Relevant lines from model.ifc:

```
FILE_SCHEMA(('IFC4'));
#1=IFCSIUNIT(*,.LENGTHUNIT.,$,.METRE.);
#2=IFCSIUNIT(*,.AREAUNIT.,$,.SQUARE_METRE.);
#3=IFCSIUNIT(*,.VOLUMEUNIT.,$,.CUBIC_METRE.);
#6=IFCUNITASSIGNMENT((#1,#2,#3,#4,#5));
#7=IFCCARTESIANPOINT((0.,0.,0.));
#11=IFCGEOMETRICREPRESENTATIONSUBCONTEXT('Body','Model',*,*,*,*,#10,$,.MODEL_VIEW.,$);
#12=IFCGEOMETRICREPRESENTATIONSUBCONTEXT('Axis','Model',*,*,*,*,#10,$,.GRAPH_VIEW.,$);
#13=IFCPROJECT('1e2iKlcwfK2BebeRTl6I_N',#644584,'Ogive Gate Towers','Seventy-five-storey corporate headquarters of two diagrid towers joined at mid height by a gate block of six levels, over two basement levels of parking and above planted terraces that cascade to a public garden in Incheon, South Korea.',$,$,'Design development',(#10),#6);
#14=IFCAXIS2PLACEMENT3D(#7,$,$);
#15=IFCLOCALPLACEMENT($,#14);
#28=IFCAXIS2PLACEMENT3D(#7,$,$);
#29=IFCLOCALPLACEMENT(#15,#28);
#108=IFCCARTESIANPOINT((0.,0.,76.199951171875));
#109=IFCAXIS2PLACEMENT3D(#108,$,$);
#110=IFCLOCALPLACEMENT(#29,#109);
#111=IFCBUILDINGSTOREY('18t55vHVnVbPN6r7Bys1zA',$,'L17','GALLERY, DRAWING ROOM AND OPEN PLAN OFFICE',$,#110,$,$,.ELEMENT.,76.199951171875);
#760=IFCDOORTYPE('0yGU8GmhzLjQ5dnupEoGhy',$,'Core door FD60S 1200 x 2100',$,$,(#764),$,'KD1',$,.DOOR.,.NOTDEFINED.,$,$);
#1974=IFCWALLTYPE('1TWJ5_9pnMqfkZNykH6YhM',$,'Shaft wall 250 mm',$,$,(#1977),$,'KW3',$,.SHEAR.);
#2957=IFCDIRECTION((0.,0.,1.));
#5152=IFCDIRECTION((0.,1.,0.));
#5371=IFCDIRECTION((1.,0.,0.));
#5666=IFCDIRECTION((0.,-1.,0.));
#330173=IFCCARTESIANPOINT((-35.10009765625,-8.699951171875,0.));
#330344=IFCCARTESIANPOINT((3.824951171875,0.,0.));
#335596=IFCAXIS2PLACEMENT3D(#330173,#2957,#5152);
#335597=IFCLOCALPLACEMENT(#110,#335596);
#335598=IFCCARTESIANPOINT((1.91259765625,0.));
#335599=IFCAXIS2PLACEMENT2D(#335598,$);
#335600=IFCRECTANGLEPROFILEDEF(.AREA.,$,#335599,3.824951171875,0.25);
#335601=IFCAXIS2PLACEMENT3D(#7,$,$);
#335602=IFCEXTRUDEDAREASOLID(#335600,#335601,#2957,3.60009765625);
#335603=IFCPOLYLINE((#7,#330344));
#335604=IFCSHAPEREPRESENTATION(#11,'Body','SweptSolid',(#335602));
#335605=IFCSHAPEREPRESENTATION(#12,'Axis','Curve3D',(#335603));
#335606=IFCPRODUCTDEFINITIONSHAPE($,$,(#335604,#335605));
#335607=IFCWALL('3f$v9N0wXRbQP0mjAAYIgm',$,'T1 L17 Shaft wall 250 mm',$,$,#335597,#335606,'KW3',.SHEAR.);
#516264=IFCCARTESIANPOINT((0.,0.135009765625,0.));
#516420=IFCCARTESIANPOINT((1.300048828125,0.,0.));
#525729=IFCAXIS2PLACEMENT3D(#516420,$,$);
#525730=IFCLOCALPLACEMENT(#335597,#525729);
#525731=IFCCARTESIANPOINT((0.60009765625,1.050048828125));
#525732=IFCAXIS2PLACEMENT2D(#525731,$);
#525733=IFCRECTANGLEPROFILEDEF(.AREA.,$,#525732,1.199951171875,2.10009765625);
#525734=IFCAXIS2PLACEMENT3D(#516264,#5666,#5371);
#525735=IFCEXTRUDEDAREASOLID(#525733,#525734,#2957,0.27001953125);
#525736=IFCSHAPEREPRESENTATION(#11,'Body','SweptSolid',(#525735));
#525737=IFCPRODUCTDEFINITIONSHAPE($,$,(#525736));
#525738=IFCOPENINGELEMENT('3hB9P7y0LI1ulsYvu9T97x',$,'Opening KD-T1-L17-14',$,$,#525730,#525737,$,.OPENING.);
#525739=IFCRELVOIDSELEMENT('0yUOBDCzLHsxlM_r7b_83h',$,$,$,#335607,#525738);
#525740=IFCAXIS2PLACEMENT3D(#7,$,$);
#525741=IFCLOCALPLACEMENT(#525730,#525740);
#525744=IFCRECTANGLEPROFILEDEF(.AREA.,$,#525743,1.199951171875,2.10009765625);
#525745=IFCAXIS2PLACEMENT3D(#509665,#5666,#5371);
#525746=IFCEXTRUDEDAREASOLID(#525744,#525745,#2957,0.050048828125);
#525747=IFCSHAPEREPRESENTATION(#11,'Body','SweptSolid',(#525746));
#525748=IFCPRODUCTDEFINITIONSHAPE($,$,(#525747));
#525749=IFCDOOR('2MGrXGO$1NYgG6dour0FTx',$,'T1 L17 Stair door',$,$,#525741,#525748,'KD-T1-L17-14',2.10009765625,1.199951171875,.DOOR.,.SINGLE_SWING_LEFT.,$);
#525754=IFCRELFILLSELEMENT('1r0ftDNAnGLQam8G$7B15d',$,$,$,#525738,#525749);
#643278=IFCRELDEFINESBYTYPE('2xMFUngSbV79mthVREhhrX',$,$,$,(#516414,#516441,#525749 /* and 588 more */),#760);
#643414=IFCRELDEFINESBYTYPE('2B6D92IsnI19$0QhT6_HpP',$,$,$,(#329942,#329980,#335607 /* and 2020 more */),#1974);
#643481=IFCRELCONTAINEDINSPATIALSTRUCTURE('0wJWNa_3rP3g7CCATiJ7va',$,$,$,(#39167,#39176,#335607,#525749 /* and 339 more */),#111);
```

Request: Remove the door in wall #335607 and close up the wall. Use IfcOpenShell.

```python
import ifcopenshell
import ifcopenshell.api.feature
import ifcopenshell.api.root
import ifcopenshell.geom
import ifcopenshell.util.shape

model = ifcopenshell.open("model.ifc")
settings = ifcopenshell.geom.settings()


def volume(element):
    """Net volume in cubic metres, openings subtracted."""
    shape = ifcopenshell.geom.create_shape(settings, element)
    return ifcopenshell.util.shape.get_volume(shape.geometry)


door = model.by_guid("2MGrXGO$1NYgG6dour0FTx")
opening = door.FillsVoids[0].RelatingOpeningElement
wall = opening.VoidsElements[0].RelatingBuildingElement
before = volume(wall)

ifcopenshell.api.root.remove_product(model, product=door)
ifcopenshell.api.feature.remove_feature(model, feature=opening)

after = volume(wall)

print(f"wall volume {before:.3f} -> {after:.3f} m3")

model.write("model_edited.ifc")
```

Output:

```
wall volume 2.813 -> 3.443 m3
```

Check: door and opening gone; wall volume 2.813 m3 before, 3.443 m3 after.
